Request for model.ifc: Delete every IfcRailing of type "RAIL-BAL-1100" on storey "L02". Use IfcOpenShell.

First a look at what the model holds.

```python
import ifcopenshell
import ifcopenshell.util.element

model = ifcopenshell.open("model.ifc")
print(model.schema)
storey = next(s for s in model.by_type("IfcBuildingStorey") if s.Name == "L02")
railings = [e for e in ifcopenshell.util.element.get_decomposition(storey) if e.is_a("IfcRailing")]
seen = {}
for e in railings:
    element_type = ifcopenshell.util.element.get_type(e)
    name = element_type.Name if element_type not in (None, e) else None
    seen[name] = seen.get(name, 0) + 1
for name, count in sorted(seen.items(), key=str):
    print(count, "x", name)
```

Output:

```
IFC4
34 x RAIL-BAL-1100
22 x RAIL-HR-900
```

```python
import ifcopenshell
import ifcopenshell.api.root
import ifcopenshell.util.element

model = ifcopenshell.open("model.ifc")

storey = next(s for s in model.by_type("IfcBuildingStorey") if s.Name == "L02")
railings = [e for e in ifcopenshell.util.element.get_decomposition(storey) if e.is_a("IfcRailing")]
targets = [e for e in railings if (t := ifcopenshell.util.element.get_type(e)) not in (None, e) and t.Name == "RAIL-BAL-1100"]

for e in targets:
    ifcopenshell.api.root.remove_product(model, product=e)
print(len(targets), "removed")

model.write("model-out.ifc")
```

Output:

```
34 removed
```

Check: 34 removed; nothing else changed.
